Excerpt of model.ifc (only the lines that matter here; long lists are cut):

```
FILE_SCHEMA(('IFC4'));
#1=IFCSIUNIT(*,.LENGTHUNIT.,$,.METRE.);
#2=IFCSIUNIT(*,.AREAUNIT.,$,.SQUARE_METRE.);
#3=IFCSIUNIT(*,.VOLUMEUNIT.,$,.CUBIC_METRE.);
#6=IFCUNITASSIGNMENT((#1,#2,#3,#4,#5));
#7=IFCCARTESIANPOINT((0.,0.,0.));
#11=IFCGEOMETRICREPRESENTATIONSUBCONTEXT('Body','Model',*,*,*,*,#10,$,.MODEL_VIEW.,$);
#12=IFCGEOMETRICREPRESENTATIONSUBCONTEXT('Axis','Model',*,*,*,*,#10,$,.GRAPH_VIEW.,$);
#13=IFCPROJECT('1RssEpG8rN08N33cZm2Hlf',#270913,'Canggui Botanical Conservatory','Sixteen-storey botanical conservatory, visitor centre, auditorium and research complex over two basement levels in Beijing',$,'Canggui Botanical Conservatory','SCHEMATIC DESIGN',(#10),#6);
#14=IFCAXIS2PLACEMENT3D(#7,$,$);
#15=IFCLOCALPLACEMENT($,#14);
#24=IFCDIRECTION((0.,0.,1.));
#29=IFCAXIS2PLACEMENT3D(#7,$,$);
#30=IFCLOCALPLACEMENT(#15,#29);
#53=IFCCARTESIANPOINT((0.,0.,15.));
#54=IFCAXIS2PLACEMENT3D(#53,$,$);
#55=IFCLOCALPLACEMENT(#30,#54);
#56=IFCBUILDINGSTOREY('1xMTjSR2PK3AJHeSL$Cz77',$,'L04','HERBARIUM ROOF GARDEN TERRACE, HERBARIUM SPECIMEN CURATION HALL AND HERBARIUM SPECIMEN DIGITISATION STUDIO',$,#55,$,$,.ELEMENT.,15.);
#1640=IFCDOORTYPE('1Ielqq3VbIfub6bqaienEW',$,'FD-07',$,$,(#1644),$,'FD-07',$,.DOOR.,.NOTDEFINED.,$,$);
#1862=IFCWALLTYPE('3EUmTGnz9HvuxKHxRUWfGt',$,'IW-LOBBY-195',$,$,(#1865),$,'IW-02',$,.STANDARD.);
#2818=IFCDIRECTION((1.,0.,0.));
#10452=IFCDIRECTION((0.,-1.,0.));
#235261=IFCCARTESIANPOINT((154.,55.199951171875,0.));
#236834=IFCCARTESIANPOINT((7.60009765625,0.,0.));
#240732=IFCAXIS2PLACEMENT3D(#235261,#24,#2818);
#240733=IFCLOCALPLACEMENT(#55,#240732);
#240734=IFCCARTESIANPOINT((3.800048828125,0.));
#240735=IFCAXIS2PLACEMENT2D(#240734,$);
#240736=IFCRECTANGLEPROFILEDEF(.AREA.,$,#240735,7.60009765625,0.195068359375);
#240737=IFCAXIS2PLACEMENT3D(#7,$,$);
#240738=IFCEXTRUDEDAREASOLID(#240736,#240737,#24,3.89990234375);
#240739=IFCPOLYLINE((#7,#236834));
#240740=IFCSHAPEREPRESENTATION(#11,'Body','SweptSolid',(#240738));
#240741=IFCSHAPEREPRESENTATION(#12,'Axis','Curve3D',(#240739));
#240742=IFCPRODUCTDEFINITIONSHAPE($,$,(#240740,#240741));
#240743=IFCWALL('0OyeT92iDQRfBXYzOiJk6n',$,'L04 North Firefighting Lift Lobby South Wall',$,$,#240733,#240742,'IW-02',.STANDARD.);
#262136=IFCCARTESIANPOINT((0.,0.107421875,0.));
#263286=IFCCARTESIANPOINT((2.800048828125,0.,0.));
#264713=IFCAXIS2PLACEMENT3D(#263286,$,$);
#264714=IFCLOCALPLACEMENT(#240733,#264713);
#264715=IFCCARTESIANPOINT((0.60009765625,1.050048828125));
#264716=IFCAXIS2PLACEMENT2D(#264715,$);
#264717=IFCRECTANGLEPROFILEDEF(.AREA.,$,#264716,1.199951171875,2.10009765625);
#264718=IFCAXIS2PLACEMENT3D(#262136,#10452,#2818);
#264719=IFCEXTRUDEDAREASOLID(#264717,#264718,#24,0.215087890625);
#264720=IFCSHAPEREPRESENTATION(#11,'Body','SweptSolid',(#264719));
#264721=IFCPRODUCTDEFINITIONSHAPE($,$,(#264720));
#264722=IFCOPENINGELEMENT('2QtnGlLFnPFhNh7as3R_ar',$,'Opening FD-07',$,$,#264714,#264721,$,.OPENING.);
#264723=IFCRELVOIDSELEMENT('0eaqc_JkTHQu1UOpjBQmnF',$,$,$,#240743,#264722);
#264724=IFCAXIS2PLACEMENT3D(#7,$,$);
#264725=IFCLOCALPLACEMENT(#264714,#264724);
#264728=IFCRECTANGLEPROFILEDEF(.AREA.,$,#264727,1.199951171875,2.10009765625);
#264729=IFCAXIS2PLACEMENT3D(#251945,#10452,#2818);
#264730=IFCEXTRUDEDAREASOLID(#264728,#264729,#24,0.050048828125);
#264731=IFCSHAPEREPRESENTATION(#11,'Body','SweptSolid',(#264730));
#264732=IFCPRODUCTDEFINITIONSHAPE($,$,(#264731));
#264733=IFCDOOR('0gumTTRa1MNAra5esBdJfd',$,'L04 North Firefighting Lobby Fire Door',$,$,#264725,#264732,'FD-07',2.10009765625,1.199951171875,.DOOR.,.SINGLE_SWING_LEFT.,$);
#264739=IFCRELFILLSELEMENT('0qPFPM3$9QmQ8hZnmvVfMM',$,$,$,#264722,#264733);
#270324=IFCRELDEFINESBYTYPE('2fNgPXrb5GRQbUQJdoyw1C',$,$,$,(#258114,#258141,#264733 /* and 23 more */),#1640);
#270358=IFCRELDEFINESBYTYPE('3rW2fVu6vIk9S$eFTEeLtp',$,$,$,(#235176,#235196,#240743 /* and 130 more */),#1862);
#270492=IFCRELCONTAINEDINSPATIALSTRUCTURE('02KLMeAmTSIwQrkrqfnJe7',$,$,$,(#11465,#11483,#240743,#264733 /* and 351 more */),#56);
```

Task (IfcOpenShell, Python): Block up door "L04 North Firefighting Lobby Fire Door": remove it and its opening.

```python
import ifcopenshell
import ifcopenshell.api.feature
import ifcopenshell.api.root
import ifcopenshell.geom
import ifcopenshell.util.shape

model = ifcopenshell.open("model.ifc")
settings = ifcopenshell.geom.settings()


def volume(element):
    """Net volume in cubic metres, openings subtracted."""
    shape = ifcopenshell.geom.create_shape(settings, element)
    return ifcopenshell.util.shape.get_volume(shape.geometry)


door = model.by_guid("0gumTTRa1MNAra5esBdJfd")
opening = door.FillsVoids[0].RelatingOpeningElement
wall = opening.VoidsElements[0].RelatingBuildingElement
before = volume(wall)

ifcopenshell.api.root.remove_product(model, product=door)
ifcopenshell.api.feature.remove_feature(model, feature=opening)

after = volume(wall)

print(f"wall volume {before:.3f} -> {after:.3f} m3")

model.write("model_updated.ifc")
```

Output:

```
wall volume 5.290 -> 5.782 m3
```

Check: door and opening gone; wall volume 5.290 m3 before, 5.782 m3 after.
